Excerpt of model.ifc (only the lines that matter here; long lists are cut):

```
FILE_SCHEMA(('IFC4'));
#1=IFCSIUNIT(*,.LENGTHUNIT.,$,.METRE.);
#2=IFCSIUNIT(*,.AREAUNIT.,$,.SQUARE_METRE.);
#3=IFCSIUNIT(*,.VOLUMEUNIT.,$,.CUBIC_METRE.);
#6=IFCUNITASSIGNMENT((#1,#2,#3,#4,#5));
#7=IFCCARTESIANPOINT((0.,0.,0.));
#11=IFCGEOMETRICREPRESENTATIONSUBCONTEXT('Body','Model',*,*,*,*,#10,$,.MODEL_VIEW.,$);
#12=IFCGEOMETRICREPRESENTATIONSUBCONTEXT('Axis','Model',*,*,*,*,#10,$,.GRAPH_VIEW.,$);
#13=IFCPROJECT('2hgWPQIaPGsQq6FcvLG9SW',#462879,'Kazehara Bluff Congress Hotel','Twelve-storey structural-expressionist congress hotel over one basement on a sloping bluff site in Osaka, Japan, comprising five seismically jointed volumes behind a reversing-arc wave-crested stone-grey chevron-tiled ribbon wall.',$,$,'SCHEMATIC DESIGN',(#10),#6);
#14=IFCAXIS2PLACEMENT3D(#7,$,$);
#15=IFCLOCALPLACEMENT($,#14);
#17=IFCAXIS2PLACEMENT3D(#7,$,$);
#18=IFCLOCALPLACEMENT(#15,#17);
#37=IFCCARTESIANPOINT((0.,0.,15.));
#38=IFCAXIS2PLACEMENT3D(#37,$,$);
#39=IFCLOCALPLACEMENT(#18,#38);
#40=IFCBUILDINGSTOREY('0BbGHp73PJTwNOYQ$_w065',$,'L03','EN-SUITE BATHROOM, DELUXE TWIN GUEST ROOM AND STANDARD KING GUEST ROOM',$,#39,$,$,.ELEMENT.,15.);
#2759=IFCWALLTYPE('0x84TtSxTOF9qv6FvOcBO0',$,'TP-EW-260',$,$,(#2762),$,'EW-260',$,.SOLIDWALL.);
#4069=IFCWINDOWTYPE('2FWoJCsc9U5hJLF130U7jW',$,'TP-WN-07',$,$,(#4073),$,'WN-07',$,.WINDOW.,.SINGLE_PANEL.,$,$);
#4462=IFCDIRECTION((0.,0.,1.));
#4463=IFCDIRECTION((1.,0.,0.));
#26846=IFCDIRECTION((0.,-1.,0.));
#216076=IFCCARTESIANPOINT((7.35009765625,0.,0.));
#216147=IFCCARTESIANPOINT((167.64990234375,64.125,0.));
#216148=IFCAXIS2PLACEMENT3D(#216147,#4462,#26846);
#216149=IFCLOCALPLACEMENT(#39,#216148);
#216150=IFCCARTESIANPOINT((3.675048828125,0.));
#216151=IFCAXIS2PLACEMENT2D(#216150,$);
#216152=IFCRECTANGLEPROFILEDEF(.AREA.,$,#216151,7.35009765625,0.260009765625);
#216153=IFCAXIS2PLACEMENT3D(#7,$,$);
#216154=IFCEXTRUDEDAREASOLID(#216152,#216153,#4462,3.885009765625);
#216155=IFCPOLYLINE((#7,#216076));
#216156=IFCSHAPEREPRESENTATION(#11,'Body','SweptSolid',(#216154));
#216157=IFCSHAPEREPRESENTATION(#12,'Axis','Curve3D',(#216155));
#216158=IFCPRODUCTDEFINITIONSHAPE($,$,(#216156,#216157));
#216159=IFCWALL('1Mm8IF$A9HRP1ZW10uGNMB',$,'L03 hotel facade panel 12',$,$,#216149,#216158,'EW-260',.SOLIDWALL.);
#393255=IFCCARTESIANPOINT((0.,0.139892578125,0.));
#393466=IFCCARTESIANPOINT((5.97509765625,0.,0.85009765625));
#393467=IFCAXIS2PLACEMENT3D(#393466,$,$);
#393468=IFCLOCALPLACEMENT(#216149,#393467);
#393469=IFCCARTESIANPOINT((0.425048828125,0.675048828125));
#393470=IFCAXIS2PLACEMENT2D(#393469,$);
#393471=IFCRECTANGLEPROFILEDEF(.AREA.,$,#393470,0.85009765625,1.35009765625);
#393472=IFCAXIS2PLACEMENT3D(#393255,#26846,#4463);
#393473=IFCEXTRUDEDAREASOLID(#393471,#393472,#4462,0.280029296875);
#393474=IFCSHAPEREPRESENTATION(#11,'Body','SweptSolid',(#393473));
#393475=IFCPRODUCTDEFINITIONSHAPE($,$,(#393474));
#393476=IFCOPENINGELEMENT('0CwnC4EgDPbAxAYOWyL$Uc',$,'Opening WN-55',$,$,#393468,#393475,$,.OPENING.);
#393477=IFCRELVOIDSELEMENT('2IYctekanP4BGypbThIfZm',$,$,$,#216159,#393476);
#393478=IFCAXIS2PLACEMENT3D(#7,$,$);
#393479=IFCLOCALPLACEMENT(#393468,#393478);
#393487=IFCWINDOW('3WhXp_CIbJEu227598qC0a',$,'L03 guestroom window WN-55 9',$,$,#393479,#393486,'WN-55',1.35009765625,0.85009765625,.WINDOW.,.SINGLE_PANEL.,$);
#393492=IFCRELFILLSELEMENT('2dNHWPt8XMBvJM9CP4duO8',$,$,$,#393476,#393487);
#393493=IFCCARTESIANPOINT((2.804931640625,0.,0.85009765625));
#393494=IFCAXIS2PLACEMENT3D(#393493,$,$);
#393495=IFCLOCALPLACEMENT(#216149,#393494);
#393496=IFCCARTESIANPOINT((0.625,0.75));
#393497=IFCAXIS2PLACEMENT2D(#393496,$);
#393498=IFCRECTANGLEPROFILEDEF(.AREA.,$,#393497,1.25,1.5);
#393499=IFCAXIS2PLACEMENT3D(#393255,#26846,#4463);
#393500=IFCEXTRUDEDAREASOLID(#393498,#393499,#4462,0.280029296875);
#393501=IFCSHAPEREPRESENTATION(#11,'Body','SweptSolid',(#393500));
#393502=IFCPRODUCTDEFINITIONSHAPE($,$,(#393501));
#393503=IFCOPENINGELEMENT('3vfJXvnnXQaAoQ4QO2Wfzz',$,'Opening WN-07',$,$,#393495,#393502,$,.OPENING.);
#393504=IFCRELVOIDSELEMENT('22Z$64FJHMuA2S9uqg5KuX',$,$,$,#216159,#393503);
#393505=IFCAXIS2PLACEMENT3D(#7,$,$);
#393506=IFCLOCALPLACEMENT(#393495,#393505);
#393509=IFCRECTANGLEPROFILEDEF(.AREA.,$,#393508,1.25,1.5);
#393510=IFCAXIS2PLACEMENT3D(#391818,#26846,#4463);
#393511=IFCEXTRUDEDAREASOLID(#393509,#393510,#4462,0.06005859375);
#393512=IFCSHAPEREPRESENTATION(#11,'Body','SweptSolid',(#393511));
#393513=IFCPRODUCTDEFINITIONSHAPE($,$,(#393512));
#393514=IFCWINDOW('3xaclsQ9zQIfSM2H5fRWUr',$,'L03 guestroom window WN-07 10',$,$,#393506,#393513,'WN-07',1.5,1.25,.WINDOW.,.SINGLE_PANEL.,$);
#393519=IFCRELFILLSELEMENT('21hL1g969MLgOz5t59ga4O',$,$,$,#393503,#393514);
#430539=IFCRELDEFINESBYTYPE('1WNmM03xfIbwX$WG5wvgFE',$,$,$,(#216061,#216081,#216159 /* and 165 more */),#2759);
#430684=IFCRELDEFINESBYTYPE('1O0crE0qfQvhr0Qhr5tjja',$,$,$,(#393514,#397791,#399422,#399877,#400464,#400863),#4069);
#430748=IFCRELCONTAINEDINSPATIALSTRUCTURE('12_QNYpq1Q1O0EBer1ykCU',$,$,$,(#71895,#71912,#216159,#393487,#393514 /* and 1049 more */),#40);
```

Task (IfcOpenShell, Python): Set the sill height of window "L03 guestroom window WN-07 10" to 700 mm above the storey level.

```python
import numpy as np
import ifcopenshell
import ifcopenshell.api.geometry
import ifcopenshell.geom
import ifcopenshell.util.element
import ifcopenshell.util.placement
import ifcopenshell.util.shape
import ifcopenshell.util.unit

model = ifcopenshell.open("model.ifc")
unit_scale = ifcopenshell.util.unit.calculate_unit_scale(model)

window = model.by_id(393514)
opening = window.FillsVoids[0].RelatingOpeningElement
storey = ifcopenshell.util.element.get_container(window, ifc_class="IfcBuildingStorey")
level = ifcopenshell.util.placement.get_local_placement(storey.ObjectPlacement)[2, 3]

# The opening's origin need not be at the sill, so measure its lowest point.
shape = ifcopenshell.geom.create_shape(ifcopenshell.geom.settings(), opening)
bottom = ifcopenshell.util.shape.get_shape_bottom_elevation(shape, shape.geometry) / unit_scale
dz = level + 0.7 / unit_scale - bottom

shift = np.array([0.0, 0.0, dz])
# The window is placed relative to its opening, so it follows when the opening moves.
matrix = ifcopenshell.util.placement.get_local_placement(opening.ObjectPlacement)
matrix[:3, 3] += shift
ifcopenshell.api.geometry.edit_object_placement(
    model, product=opening, matrix=matrix, is_si=False, should_transform_children=True
)

print(f"moved by {dz * unit_scale:+.3f} m")

model.write("model-out.ifc")
```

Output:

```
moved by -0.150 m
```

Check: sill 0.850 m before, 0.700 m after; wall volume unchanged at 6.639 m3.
